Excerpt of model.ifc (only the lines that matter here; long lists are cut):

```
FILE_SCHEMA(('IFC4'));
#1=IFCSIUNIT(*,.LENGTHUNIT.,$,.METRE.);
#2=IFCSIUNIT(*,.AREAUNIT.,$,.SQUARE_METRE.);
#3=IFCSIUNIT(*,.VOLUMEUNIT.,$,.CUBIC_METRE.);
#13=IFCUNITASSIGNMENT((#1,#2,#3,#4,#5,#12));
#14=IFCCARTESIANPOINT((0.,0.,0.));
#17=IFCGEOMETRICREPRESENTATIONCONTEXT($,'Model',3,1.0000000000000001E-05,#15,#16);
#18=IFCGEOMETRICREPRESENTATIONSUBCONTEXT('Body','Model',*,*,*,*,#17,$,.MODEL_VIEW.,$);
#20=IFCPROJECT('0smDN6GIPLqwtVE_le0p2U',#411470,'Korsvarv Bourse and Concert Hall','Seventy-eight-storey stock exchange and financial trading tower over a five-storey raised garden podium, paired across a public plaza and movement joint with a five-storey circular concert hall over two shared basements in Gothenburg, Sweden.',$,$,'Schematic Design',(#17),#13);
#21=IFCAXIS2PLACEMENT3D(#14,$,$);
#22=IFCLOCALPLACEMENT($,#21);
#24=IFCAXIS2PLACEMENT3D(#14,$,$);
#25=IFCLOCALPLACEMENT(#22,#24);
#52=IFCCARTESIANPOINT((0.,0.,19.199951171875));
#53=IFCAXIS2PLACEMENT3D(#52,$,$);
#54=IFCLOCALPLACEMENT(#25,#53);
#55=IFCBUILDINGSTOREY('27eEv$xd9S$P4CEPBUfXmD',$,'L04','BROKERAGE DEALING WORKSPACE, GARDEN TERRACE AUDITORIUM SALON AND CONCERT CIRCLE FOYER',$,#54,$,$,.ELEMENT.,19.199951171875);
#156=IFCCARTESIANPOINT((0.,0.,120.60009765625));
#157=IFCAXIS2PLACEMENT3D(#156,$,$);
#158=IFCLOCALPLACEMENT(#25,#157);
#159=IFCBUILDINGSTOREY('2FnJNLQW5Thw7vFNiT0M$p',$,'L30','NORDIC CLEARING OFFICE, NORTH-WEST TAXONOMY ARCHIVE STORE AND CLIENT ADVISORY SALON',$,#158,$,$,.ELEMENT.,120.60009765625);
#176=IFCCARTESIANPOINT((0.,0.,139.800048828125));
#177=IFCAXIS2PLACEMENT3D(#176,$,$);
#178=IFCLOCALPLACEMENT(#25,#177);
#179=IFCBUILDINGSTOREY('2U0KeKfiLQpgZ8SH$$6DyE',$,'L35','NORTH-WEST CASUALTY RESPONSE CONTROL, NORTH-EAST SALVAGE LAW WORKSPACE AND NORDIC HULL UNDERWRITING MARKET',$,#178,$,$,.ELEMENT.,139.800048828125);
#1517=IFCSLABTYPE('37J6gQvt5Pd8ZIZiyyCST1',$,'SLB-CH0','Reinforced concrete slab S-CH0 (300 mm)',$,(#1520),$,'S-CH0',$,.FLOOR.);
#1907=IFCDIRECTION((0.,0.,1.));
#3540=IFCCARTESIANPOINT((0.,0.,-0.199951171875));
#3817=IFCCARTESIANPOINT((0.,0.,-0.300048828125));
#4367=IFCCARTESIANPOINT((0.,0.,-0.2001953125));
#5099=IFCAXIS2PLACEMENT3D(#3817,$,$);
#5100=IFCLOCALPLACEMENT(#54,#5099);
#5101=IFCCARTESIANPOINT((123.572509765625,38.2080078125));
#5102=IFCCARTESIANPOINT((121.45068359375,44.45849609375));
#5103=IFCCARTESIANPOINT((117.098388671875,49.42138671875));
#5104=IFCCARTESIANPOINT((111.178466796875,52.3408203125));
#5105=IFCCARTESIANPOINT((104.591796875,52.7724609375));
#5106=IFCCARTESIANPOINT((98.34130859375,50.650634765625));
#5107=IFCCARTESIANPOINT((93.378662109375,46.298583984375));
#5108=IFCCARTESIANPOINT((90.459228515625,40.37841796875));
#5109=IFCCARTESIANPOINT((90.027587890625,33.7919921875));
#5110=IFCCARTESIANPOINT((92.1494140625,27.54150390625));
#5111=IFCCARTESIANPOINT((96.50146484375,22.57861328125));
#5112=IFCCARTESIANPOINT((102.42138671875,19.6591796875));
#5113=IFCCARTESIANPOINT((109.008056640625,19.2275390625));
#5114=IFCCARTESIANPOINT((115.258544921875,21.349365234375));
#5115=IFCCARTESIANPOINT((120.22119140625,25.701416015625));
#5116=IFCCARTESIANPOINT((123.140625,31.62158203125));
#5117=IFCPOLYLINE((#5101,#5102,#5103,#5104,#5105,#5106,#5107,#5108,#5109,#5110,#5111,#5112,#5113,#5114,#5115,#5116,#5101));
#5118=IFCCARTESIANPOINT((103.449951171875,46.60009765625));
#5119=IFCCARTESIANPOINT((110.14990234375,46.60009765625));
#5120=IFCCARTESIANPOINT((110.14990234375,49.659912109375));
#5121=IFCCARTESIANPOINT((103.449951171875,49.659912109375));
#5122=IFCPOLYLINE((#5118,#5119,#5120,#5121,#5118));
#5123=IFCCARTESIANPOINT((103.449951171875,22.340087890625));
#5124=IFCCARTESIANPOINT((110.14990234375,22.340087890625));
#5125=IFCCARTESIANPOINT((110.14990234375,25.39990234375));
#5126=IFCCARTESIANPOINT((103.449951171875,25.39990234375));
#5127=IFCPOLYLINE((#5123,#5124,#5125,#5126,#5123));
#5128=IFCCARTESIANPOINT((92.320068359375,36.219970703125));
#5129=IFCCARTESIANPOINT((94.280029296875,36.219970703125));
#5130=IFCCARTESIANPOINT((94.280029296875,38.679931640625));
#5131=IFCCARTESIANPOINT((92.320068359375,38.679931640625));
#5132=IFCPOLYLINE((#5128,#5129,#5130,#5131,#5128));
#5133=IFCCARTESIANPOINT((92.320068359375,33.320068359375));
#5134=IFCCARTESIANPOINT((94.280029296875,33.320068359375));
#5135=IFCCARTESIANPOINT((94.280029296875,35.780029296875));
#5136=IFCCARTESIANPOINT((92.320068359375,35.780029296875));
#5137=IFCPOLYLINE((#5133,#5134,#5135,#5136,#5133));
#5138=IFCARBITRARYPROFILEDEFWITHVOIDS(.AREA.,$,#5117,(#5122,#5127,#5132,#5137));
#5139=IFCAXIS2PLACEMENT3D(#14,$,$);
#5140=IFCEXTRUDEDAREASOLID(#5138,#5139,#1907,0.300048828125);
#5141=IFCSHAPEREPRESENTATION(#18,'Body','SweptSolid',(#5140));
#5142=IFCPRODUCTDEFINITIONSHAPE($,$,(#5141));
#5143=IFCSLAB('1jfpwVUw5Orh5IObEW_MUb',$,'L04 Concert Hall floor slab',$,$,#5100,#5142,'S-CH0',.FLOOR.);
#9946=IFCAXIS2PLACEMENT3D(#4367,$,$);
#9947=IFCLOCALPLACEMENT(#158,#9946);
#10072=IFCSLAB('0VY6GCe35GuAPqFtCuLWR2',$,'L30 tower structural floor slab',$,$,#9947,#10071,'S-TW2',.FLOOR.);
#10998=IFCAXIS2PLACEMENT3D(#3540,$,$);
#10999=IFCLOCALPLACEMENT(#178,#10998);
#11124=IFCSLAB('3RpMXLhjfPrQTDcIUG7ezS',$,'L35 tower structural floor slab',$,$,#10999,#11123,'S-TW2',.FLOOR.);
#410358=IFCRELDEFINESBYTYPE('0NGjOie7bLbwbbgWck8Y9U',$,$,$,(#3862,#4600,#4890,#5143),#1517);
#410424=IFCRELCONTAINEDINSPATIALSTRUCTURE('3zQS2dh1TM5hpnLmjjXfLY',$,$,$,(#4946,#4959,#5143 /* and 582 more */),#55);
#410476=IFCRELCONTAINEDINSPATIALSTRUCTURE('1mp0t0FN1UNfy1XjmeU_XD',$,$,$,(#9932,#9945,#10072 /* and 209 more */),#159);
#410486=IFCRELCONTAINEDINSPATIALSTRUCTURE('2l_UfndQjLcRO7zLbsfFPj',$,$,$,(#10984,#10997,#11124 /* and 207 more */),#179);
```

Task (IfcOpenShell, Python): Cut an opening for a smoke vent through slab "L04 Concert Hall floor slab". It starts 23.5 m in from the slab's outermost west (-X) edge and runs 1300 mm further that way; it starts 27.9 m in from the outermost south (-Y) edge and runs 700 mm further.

```python
import numpy as np
import ifcopenshell
import ifcopenshell.api.feature
import ifcopenshell.api.geometry
import ifcopenshell.api.root
import ifcopenshell.geom
import ifcopenshell.util.placement
import ifcopenshell.util.representation
import ifcopenshell.util.shape
import ifcopenshell.util.unit

model = ifcopenshell.open("model.ifc")
unit_scale = ifcopenshell.util.unit.calculate_unit_scale(model)
settings = ifcopenshell.geom.settings()


def volume(element):
    """Net volume in cubic metres, openings subtracted."""
    shape = ifcopenshell.geom.create_shape(settings, element)
    return ifcopenshell.util.shape.get_volume(shape.geometry)


slab = model.by_guid("1jfpwVUw5Orh5IObEW_MUb")
before = volume(slab)

# Extent in the slab's own axes, in metres. The edges named are its -X and -Y sides.
slab_shape = ifcopenshell.geom.create_shape(settings, slab)
vertices = ifcopenshell.util.shape.get_vertices(slab_shape.geometry)
x_min, y_min, bottom = vertices.min(axis=0)
top = vertices[:, 2].max()

opening = ifcopenshell.api.root.create_entity(model, ifc_class="IfcOpeningElement", name="Smoke vent opening", predefined_type="OPENING")
context = ifcopenshell.util.representation.get_context(model, "Model", "Body", "MODEL_VIEW")
width, depth = 1.3, 0.7
outline = [(0.0, 0.0), (width, 0.0), (width, depth), (0.0, depth), (0.0, 0.0)]
# Overshoot both faces by 50 mm so the cut is clean.
shape = ifcopenshell.api.geometry.add_slab_representation(
    model, context=context, depth=top - bottom + 0.1, polyline=outline
)
ifcopenshell.api.geometry.assign_representation(model, product=opening, representation=shape)

matrix = ifcopenshell.util.placement.get_local_placement(slab.ObjectPlacement)
matrix[:, 3] = matrix @ np.append(np.array([x_min + 23.5, y_min + 27.9, bottom - 0.05]) / unit_scale, 1.0)
ifcopenshell.api.geometry.edit_object_placement(model, product=opening, matrix=matrix, is_si=False)
ifcopenshell.api.feature.add_feature(model, feature=opening, element=slab)

after = volume(slab)

print(f"slab volume {before:.3f} -> {after:.3f} m3")

model.write("model_rev.ifc")
```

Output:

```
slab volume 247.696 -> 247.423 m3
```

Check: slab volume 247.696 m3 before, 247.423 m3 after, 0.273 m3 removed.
